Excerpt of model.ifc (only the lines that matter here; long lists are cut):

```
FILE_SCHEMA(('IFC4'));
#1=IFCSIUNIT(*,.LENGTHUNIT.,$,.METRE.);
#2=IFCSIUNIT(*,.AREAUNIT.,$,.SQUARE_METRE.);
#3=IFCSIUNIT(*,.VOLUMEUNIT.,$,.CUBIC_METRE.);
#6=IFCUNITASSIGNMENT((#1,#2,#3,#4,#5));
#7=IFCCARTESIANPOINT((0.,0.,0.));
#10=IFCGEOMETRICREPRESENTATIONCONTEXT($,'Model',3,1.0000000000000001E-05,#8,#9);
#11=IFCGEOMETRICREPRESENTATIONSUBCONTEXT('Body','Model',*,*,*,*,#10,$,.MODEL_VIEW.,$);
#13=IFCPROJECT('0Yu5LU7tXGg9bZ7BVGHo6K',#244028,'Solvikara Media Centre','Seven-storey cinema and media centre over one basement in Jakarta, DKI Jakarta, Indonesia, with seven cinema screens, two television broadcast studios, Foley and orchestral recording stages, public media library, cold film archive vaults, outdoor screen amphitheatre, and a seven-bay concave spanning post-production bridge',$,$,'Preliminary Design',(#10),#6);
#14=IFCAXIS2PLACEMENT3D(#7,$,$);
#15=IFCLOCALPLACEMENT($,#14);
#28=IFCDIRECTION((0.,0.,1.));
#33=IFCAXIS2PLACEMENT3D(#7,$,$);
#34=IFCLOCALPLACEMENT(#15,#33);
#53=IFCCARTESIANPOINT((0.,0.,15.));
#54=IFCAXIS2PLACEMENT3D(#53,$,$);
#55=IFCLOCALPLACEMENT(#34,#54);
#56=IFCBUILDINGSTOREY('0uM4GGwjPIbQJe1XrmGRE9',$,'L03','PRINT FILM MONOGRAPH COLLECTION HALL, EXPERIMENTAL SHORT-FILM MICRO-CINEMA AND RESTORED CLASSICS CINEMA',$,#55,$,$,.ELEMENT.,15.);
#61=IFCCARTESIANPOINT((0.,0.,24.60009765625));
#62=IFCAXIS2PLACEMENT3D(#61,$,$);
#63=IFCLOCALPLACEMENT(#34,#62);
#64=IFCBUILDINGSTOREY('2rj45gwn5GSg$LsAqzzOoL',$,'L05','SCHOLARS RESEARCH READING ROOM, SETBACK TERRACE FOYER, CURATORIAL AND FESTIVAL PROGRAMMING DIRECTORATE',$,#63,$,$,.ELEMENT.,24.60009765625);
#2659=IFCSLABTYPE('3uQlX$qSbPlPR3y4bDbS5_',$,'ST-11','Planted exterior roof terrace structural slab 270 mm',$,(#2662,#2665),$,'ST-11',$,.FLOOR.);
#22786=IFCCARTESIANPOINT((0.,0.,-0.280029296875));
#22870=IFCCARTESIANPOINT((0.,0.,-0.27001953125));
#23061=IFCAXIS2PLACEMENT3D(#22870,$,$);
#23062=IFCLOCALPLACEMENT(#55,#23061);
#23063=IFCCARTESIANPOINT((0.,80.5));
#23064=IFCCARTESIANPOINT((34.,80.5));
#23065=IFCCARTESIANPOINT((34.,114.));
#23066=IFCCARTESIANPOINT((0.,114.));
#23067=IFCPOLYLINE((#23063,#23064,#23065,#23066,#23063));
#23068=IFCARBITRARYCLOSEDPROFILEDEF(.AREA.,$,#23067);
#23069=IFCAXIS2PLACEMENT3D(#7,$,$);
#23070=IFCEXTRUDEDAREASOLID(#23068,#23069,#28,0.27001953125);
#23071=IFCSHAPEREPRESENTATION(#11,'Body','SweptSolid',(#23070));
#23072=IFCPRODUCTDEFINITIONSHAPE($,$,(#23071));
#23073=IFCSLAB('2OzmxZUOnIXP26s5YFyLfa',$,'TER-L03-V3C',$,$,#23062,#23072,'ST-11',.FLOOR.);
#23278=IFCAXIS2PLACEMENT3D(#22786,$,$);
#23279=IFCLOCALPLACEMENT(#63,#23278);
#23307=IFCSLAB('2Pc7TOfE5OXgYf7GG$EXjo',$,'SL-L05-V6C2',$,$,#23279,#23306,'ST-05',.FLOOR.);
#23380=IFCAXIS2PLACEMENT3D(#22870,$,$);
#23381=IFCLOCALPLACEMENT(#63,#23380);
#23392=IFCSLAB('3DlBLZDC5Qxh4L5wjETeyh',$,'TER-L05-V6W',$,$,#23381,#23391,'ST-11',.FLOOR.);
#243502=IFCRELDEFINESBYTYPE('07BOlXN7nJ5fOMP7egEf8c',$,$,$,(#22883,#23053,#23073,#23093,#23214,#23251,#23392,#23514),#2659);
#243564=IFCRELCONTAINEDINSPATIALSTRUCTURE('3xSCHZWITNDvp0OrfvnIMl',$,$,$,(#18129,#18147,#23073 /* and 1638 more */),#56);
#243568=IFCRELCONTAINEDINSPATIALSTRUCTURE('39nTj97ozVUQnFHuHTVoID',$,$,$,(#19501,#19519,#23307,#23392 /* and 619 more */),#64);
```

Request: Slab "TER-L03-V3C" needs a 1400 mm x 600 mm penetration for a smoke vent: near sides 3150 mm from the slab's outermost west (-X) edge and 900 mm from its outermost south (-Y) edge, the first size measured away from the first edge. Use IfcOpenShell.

```python
import numpy as np
import ifcopenshell
import ifcopenshell.api.feature
import ifcopenshell.api.geometry
import ifcopenshell.api.root
import ifcopenshell.geom
import ifcopenshell.util.placement
import ifcopenshell.util.representation
import ifcopenshell.util.shape
import ifcopenshell.util.unit

model = ifcopenshell.open("model.ifc")
unit_scale = ifcopenshell.util.unit.calculate_unit_scale(model)
settings = ifcopenshell.geom.settings()


def volume(element):
    """Net volume in cubic metres, openings subtracted."""
    shape = ifcopenshell.geom.create_shape(settings, element)
    return ifcopenshell.util.shape.get_volume(shape.geometry)


slab = model.by_guid("2OzmxZUOnIXP26s5YFyLfa")
before = volume(slab)

# Extent in the slab's own axes, in metres. The edges named are its -X and -Y sides.
slab_shape = ifcopenshell.geom.create_shape(settings, slab)
vertices = ifcopenshell.util.shape.get_vertices(slab_shape.geometry)
x_min, y_min, bottom = vertices.min(axis=0)
top = vertices[:, 2].max()

opening = ifcopenshell.api.root.create_entity(model, ifc_class="IfcOpeningElement", name="Smoke vent opening", predefined_type="OPENING")
context = ifcopenshell.util.representation.get_context(model, "Model", "Body", "MODEL_VIEW")
width, depth = 1.4, 0.6
outline = [(0.0, 0.0), (width, 0.0), (width, depth), (0.0, depth), (0.0, 0.0)]
# Overshoot both faces by 50 mm so the cut is clean.
shape = ifcopenshell.api.geometry.add_slab_representation(
    model, context=context, depth=top - bottom + 0.1, polyline=outline
)
ifcopenshell.api.geometry.assign_representation(model, product=opening, representation=shape)

matrix = ifcopenshell.util.placement.get_local_placement(slab.ObjectPlacement)
matrix[:, 3] = matrix @ np.append(np.array([x_min + 3.15, y_min + 0.9, bottom - 0.05]) / unit_scale, 1.0)
ifcopenshell.api.geometry.edit_object_placement(model, product=opening, matrix=matrix, is_si=False)
ifcopenshell.api.feature.add_feature(model, feature=opening, element=slab)

after = volume(slab)

print(f"slab volume {before:.3f} -> {after:.3f} m3")

model.write("model_rev.ifc")
```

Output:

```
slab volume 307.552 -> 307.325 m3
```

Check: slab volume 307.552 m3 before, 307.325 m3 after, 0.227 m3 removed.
